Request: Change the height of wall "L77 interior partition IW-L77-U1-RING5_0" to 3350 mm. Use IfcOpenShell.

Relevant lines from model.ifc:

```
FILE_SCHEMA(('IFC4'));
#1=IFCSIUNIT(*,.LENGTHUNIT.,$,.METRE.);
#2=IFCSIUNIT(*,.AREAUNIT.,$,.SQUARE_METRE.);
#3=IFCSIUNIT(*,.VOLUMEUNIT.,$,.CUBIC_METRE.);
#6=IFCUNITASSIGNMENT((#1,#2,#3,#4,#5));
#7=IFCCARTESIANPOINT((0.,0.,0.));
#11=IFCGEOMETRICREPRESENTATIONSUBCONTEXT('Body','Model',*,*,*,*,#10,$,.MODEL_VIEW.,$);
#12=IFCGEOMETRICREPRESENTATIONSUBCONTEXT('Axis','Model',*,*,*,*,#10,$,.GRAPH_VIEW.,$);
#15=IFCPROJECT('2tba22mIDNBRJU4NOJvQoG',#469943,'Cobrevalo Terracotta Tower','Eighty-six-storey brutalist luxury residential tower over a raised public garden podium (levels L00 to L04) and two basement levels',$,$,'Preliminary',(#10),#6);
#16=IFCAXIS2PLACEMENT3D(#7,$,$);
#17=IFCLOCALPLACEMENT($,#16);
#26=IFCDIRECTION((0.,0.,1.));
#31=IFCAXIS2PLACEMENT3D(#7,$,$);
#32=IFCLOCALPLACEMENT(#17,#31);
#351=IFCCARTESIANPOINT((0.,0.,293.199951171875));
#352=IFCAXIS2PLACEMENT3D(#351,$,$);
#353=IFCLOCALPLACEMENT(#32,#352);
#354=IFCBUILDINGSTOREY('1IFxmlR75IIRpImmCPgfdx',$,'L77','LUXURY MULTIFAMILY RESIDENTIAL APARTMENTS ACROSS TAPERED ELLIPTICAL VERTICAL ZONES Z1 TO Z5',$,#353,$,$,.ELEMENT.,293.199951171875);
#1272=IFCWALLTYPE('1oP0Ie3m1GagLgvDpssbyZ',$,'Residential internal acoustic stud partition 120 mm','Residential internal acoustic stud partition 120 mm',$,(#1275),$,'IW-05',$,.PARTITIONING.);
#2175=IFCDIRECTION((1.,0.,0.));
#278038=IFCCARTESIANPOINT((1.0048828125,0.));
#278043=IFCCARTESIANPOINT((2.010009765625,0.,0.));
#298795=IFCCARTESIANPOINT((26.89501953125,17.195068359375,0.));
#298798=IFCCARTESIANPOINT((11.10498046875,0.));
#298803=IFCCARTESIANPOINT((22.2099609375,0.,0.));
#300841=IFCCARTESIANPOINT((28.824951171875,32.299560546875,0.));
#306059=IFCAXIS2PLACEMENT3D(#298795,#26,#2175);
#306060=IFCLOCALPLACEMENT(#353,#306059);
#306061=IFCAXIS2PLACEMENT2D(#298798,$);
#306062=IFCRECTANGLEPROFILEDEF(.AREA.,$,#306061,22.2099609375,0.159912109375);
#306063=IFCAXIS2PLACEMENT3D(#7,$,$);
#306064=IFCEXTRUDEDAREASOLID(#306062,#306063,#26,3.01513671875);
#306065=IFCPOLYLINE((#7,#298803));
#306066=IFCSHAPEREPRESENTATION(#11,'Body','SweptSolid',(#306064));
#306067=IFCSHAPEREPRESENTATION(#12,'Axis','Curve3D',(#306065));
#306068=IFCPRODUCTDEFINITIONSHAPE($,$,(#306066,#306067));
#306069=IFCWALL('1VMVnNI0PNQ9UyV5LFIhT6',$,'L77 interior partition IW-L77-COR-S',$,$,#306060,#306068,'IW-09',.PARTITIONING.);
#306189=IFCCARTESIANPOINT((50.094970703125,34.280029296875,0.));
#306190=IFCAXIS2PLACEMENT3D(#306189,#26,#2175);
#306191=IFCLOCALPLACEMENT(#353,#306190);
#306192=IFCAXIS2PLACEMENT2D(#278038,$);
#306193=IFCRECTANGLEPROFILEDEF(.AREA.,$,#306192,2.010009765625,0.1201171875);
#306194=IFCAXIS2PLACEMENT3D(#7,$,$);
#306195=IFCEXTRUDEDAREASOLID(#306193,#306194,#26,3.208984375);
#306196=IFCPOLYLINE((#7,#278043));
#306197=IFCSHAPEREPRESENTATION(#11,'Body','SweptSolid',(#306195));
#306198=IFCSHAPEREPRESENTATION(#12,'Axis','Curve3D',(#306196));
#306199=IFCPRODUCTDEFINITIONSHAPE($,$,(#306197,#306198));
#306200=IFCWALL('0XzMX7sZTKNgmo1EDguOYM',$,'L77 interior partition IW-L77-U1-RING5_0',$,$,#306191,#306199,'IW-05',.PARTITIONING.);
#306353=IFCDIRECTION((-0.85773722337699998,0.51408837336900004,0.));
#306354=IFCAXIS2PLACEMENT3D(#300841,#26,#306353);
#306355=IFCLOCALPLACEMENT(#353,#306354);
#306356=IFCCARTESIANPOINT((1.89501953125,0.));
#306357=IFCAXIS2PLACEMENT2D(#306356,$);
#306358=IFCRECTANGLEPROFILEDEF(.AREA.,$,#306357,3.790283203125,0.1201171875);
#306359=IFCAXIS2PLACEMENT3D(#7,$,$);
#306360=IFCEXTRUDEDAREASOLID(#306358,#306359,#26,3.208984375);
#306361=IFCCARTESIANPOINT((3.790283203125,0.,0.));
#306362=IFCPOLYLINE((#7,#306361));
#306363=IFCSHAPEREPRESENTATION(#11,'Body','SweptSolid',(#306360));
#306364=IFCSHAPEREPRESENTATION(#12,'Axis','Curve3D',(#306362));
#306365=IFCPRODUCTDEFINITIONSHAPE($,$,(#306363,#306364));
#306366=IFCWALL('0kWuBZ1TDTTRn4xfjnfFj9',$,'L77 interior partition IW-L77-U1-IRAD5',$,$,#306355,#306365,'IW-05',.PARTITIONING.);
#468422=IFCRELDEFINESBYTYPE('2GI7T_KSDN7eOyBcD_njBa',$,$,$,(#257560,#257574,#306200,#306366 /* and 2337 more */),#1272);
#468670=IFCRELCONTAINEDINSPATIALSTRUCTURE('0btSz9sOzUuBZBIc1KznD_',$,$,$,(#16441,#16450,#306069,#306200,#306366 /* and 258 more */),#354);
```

```python
import ifcopenshell
import ifcopenshell.geom
import ifcopenshell.util.representation
import ifcopenshell.util.shape

model = ifcopenshell.open("model.ifc")
settings = ifcopenshell.geom.settings()


def volume(element):
    """Net volume in cubic metres, openings subtracted."""
    shape = ifcopenshell.geom.create_shape(settings, element)
    return ifcopenshell.util.shape.get_volume(shape.geometry)


wall = model.by_id(306200)
before = volume(wall)

body = ifcopenshell.util.representation.get_representation(wall, "Model", "Body")
solid = body.Items[0]
old_height = solid.Depth
solid.Depth = 3.35
after = volume(wall)

print(f"height {old_height:g} -> {solid.Depth:g}, volume {before:.3f} -> {after:.3f} m3")

model.write("model_edited.ifc")
```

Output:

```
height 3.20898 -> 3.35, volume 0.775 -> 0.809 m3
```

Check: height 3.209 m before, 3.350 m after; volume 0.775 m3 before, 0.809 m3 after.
